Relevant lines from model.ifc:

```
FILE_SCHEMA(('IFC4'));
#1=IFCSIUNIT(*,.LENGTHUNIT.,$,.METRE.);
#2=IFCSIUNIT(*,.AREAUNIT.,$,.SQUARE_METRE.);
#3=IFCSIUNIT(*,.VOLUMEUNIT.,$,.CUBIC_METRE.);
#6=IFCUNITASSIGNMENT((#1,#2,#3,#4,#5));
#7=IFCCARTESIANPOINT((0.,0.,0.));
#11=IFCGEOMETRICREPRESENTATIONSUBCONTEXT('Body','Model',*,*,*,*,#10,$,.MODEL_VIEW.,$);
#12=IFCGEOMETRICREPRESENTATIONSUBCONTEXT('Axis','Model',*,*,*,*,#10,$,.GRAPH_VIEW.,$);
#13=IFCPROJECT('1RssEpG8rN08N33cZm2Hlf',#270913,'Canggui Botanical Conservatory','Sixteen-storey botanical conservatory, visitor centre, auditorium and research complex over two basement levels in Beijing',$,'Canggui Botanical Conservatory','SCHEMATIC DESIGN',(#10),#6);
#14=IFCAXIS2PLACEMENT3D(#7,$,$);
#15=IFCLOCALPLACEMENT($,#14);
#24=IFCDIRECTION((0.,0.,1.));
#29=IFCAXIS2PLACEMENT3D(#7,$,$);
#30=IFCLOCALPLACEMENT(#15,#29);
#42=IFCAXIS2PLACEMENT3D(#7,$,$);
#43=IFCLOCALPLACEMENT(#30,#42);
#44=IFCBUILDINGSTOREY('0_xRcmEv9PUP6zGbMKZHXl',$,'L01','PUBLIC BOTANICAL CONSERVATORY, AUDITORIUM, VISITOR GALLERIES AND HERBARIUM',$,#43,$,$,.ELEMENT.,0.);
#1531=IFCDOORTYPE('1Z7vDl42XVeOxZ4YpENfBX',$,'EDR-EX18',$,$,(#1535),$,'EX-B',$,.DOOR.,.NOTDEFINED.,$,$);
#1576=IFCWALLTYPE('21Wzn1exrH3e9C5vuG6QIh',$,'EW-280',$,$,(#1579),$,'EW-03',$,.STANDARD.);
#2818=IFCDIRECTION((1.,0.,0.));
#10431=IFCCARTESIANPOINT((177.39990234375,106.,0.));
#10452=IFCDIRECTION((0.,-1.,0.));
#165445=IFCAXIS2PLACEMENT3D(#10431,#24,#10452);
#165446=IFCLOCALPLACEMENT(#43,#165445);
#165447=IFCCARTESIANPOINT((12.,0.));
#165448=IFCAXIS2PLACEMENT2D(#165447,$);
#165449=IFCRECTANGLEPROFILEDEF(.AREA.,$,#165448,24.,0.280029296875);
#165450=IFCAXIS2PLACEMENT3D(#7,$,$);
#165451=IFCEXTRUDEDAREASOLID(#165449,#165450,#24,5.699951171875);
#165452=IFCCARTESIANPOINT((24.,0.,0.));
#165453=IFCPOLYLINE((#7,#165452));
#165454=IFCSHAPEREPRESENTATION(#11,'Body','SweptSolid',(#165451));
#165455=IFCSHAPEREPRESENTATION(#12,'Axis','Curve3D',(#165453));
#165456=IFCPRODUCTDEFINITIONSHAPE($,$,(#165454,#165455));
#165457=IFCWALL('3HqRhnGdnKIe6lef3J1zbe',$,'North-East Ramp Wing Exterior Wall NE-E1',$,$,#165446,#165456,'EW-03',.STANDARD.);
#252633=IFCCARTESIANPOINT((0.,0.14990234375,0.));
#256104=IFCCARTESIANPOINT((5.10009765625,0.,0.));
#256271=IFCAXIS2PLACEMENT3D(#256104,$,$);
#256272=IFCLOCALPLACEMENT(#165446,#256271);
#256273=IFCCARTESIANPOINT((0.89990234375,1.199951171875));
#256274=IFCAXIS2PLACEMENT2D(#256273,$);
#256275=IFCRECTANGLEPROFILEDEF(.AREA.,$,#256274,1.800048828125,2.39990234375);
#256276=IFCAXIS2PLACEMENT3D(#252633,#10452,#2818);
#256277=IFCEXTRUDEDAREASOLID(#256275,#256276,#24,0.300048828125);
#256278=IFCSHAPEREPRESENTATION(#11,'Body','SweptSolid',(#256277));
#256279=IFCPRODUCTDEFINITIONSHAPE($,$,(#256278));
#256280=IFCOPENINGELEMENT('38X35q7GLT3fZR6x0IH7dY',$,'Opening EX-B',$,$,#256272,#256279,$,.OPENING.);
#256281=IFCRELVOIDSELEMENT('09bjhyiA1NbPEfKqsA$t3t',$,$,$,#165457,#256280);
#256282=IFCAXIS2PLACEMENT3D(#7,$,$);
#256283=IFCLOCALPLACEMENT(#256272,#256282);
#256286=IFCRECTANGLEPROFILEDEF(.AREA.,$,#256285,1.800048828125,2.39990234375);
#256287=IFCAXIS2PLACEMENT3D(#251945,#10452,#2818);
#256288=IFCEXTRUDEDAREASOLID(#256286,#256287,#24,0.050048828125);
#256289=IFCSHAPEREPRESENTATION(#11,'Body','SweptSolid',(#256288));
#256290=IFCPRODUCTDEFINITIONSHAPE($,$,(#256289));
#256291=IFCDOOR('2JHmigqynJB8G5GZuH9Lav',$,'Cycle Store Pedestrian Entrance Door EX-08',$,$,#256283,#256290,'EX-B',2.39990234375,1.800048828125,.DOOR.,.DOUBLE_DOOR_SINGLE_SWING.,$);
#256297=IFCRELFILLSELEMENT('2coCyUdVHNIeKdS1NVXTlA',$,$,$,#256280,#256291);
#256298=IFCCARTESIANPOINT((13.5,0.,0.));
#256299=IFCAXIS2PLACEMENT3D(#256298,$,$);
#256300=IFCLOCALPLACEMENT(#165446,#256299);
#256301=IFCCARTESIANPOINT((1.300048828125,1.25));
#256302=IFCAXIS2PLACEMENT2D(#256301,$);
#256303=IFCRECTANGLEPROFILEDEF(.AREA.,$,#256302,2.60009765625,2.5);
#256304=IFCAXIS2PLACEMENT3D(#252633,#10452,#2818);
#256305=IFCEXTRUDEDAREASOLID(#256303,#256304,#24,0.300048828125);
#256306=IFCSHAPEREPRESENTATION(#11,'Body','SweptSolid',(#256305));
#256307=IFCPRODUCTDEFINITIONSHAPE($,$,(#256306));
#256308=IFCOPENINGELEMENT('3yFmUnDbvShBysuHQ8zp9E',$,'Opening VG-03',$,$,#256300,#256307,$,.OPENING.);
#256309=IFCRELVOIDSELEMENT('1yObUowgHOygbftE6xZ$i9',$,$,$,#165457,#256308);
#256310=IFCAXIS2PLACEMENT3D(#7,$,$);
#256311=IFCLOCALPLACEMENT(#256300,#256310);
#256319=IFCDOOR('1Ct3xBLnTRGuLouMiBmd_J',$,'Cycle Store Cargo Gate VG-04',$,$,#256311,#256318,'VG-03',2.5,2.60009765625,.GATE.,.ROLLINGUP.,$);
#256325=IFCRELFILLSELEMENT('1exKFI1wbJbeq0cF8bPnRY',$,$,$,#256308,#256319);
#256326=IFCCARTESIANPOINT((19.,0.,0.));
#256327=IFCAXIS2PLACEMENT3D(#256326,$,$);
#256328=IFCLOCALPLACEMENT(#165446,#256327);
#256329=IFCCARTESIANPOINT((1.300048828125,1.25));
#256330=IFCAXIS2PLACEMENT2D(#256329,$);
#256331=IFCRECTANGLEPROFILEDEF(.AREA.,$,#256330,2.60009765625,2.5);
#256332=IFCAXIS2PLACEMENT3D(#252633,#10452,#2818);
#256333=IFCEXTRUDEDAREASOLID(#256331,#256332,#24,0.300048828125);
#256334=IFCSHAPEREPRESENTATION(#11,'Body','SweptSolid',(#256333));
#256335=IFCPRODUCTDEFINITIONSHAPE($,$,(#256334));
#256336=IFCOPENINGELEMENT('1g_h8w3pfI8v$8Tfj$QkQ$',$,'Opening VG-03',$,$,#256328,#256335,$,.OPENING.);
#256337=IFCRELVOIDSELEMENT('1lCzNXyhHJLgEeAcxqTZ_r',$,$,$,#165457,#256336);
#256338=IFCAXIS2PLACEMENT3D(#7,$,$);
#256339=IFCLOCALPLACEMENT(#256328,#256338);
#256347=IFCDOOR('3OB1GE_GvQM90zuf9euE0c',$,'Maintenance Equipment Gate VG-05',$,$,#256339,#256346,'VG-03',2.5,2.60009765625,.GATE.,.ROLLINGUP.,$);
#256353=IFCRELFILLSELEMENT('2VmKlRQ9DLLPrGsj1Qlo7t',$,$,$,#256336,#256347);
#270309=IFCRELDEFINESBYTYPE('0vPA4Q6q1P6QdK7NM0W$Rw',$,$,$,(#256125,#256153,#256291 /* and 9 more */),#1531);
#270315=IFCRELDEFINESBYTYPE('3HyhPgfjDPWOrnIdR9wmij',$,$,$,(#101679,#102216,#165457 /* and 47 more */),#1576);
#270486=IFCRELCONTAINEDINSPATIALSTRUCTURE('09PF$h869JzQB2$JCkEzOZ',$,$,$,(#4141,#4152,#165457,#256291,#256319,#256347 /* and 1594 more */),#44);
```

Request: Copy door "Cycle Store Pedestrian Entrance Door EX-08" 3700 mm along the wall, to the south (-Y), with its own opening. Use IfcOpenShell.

```python
import ifcopenshell
import ifcopenshell.api.feature
import ifcopenshell.api.geometry
import ifcopenshell.api.root
import ifcopenshell.geom
import ifcopenshell.util.element
import ifcopenshell.util.placement
import ifcopenshell.util.shape

model = ifcopenshell.open("model.ifc")
settings = ifcopenshell.geom.settings()


def volume(element):
    """Net volume in cubic metres, openings subtracted."""
    shape = ifcopenshell.geom.create_shape(settings, element)
    return ifcopenshell.util.shape.get_volume(shape.geometry)


door = model.by_id(256291)
opening = door.FillsVoids[0].RelatingOpeningElement
wall = opening.VoidsElements[0].RelatingBuildingElement
before = volume(wall)
shift = ifcopenshell.util.placement.get_local_placement(wall.ObjectPlacement)[:3, 0] * 3.7

# copy_class copies the void relationship, type, container and properties, but no geometry.
new_opening = ifcopenshell.api.root.copy_class(model, product=opening)
new_opening.Representation = ifcopenshell.util.element.copy_deep(
    model, opening.Representation, exclude=["IfcGeometricRepresentationContext", "IfcRepresentationMap"]
)
new_door = ifcopenshell.api.root.copy_class(model, product=door)
new_door.Representation = ifcopenshell.util.element.copy_deep(
    model, door.Representation, exclude=["IfcGeometricRepresentationContext", "IfcRepresentationMap"]
)
new_door.Tag = None
ifcopenshell.api.feature.add_filling(model, opening=new_opening, element=new_door)

for old, new in ((opening, new_opening), (door, new_door)):
    matrix = ifcopenshell.util.placement.get_local_placement(old.ObjectPlacement)
    matrix[:3, 3] += shift
    ifcopenshell.api.geometry.edit_object_placement(model, product=new, matrix=matrix, is_si=False)

after = volume(wall)

print(f"wall volume {before:.3f} -> {after:.3f} m3")

model.write("model-out.ifc")
```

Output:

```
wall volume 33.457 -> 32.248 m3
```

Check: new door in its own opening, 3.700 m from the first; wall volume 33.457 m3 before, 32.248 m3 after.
